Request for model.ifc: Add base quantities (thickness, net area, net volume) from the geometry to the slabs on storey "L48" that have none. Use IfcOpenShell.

First a look at what the model holds.

```python
import ifcopenshell
import ifcopenshell.util.element
import ifcopenshell.util.unit

model = ifcopenshell.open("model.ifc")
print(model.schema)
for unit_type in ("LENGTHUNIT", "AREAUNIT", "VOLUMEUNIT"):
    print(unit_type, ifcopenshell.util.unit.calculate_unit_scale(model, unit_type))
storey = next(s for s in model.by_type("IfcBuildingStorey") if s.Name == "L48")
slabs = [e for e in ifcopenshell.util.element.get_decomposition(storey) if e.is_a("IfcSlab")]
for e in sorted(slabs, key=lambda e: e.id()):
    print(e.id(), e.is_a(), e.Name, list(ifcopenshell.util.element.get_psets(e, qtos_only=True)), sep=" | ")
```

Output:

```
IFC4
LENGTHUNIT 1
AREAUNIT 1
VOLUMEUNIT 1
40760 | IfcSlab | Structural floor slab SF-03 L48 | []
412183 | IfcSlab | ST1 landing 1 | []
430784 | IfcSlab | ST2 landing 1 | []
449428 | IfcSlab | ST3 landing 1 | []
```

```python
import ifcopenshell
import ifcopenshell.api.pset
import ifcopenshell.geom
import ifcopenshell.util.element
import ifcopenshell.util.shape
import ifcopenshell.util.unit

model = ifcopenshell.open("model.ifc")
unit_scale = ifcopenshell.util.unit.calculate_unit_scale(model)
area_scale = ifcopenshell.util.unit.calculate_unit_scale(model, "AREAUNIT")
volume_scale = ifcopenshell.util.unit.calculate_unit_scale(model, "VOLUMEUNIT")
settings = ifcopenshell.geom.settings()

storey = next(s for s in model.by_type("IfcBuildingStorey") if s.Name == "L48")
slabs = [e for e in ifcopenshell.util.element.get_decomposition(storey) if e.is_a("IfcSlab")]

for e in sorted(slabs, key=lambda e: e.id()):
    if ifcopenshell.util.element.get_psets(e, qtos_only=True, should_inherit=False):
        continue
    # Geometry comes back in metres, in the element's own axes.
    shape = ifcopenshell.geom.create_shape(settings, e)
    values = {
        "Width": ifcopenshell.util.shape.get_z(shape.geometry) / unit_scale,
        "NetArea": ifcopenshell.util.shape.get_footprint_area(shape.geometry) / area_scale,
        "NetVolume": ifcopenshell.util.shape.get_volume(shape.geometry) / volume_scale,
    }
    qto = ifcopenshell.api.pset.add_qto(model, product=e, name="Qto_SlabBaseQuantities")
    ifcopenshell.api.pset.edit_qto(model, qto=qto, properties=values)
    print(e.id(), {k: round(v, 3) for k, v in values.items()})

model.write("model_v2.ifc")
```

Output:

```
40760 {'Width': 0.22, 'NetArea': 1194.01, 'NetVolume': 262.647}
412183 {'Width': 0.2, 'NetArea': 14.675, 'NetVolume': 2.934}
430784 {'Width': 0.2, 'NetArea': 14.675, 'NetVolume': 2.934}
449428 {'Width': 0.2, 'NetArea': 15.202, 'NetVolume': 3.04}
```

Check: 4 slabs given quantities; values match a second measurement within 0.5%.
